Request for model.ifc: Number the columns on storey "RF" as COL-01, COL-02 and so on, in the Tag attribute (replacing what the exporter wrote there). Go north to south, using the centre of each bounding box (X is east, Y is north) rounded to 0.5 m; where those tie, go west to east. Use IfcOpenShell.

First a look at what the model holds.

```python
import ifcopenshell
import ifcopenshell.util.element
import ifcopenshell.util.placement

model = ifcopenshell.open("model.ifc")
print(model.schema)
storey = next(s for s in model.by_type("IfcBuildingStorey") if s.Name == "RF")
columns = [e for e in ifcopenshell.util.element.get_decomposition(storey) if e.is_a("IfcColumn")]
for e in sorted(columns, key=lambda e: e.id()):
    origin = ifcopenshell.util.placement.get_local_placement(e.ObjectPlacement)[:3, 3]
    print(e.id(), e.Tag, e.Name, origin.round(2) + 0.0, sep=" | ")
```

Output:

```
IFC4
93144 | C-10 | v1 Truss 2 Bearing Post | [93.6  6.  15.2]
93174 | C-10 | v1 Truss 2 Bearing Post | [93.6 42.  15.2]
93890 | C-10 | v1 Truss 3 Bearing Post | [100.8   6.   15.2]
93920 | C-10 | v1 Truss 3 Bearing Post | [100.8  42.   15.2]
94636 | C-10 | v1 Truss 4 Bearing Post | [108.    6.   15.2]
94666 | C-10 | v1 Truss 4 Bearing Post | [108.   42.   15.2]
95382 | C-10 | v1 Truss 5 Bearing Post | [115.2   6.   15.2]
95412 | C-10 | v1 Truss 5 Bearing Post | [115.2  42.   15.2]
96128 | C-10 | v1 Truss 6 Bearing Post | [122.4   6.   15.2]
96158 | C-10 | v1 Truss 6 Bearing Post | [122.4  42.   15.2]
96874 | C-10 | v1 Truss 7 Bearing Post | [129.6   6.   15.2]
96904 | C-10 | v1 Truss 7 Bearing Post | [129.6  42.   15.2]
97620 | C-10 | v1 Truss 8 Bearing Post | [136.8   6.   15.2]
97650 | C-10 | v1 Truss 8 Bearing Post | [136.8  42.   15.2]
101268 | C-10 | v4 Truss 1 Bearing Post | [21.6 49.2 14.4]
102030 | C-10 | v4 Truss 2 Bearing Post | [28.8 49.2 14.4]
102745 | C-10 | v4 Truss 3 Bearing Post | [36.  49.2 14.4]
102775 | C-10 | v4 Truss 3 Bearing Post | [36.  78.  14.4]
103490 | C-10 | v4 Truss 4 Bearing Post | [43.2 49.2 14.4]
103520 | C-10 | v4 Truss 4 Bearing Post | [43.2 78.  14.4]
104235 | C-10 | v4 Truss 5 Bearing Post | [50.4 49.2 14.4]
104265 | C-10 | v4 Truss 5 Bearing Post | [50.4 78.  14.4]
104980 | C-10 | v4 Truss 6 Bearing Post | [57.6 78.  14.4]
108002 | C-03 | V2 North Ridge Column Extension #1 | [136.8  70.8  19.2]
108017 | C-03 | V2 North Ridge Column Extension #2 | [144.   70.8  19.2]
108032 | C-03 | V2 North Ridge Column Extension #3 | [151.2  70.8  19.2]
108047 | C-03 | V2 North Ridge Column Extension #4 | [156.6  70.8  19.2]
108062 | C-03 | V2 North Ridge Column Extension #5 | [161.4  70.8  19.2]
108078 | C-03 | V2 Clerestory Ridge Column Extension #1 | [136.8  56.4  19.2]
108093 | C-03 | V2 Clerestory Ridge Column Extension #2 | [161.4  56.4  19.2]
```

```python
import ifcopenshell
import ifcopenshell.geom
import ifcopenshell.util.element
import ifcopenshell.util.shape

model = ifcopenshell.open("model.ifc")
settings = ifcopenshell.geom.settings()
settings.set("use-world-coords", True)


def centre(element):
    shape = ifcopenshell.geom.create_shape(settings, element)
    return ifcopenshell.util.shape.get_bbox_centroid(shape.geometry)


storey = next(s for s in model.by_type("IfcBuildingStorey") if s.Name == "RF")
columns = [e for e in ifcopenshell.util.element.get_decomposition(storey) if e.is_a("IfcColumn")]

# Insertion points can sit at a corner or the storey origin, so sort by the geometry (in metres).
centres = {e: centre(e) for e in columns}
columns.sort(key=lambda e: (-round(centres[e][1] / 0.5), centres[e][0]))

for i, e in enumerate(columns, start=1):
    number = f"COL-{i:02d}"
    e.Tag = number
    print(e.id(), number)

model.write("model_v2.ifc")
```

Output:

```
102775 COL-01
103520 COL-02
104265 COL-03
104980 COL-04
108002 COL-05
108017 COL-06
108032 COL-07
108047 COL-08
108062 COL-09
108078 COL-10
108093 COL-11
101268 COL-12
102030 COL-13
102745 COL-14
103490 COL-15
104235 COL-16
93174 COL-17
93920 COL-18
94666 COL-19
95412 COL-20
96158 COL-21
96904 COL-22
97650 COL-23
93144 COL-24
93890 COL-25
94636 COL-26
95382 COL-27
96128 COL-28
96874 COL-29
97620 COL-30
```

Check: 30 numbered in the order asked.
